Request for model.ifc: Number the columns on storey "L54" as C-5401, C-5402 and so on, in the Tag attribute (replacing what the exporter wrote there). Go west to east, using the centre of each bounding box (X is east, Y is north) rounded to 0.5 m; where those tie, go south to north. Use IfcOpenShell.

First a look at what the model holds.

```python
import ifcopenshell
import ifcopenshell.util.element
import ifcopenshell.util.placement

model = ifcopenshell.open("model.ifc")
print(model.schema)
storey = next(s for s in model.by_type("IfcBuildingStorey") if s.Name == "L54")
columns = [e for e in ifcopenshell.util.element.get_decomposition(storey) if e.is_a("IfcColumn")]
for e in sorted(columns, key=lambda e: e.id()):
    origin = ifcopenshell.util.placement.get_local_placement(e.ObjectPlacement)[:3, 3]
    print(e.id(), e.Tag, e.Name, origin.round(2) + 0.0, sep=" | ")
```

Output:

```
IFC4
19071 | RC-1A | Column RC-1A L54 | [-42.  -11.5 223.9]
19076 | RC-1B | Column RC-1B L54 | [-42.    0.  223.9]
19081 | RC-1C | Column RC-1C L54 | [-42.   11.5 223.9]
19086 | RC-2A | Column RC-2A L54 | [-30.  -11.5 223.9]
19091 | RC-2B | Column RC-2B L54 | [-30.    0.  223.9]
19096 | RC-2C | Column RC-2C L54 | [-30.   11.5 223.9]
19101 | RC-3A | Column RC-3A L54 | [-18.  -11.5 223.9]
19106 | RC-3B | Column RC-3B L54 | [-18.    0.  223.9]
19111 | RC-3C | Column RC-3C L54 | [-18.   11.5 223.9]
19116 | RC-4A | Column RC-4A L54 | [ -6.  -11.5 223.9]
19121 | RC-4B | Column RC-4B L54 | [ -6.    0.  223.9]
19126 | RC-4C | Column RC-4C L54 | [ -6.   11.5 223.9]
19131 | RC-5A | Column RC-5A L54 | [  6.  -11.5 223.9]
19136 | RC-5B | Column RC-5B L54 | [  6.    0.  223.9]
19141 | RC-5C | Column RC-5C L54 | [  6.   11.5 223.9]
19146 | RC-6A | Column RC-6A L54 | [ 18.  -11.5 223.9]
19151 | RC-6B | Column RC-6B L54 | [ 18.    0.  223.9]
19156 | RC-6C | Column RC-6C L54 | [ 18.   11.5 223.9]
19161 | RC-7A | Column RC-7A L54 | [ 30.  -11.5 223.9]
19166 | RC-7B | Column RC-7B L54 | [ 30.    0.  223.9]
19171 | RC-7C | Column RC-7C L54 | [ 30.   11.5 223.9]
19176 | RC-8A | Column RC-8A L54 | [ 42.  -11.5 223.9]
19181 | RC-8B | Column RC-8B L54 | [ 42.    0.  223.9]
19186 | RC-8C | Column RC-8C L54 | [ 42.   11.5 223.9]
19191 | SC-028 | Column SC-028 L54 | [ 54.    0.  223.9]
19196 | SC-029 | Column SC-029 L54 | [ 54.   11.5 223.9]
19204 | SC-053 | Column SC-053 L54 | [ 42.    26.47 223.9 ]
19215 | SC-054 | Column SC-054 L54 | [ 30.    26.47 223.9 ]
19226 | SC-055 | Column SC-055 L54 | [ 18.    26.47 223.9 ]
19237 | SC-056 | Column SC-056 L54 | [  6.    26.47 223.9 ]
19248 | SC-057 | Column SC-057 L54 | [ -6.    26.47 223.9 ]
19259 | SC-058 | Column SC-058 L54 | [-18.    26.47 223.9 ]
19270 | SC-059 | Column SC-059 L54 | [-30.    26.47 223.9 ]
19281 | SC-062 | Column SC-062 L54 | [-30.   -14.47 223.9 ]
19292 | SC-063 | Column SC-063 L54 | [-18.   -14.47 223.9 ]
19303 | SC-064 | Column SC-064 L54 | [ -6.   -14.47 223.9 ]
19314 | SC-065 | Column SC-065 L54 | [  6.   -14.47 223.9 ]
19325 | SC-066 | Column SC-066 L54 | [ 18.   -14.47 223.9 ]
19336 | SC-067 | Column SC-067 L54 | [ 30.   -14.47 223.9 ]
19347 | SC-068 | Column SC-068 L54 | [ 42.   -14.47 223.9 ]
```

```python
import ifcopenshell
import ifcopenshell.geom
import ifcopenshell.util.element
import ifcopenshell.util.shape

model = ifcopenshell.open("model.ifc")
settings = ifcopenshell.geom.settings()
settings.set("use-world-coords", True)


def centre(element):
    shape = ifcopenshell.geom.create_shape(settings, element)
    return ifcopenshell.util.shape.get_bbox_centroid(shape.geometry)


storey = next(s for s in model.by_type("IfcBuildingStorey") if s.Name == "L54")
columns = [e for e in ifcopenshell.util.element.get_decomposition(storey) if e.is_a("IfcColumn")]

# Insertion points can sit at a corner or the storey origin, so sort by the geometry (in metres).
centres = {e: centre(e) for e in columns}
columns.sort(key=lambda e: (round(centres[e][0] / 0.5), centres[e][1]))

for i, e in enumerate(columns, start=1):
    number = f"C-54{i:02d}"
    e.Tag = number
    print(e.id(), number)

model.write("model_updated.ifc")
```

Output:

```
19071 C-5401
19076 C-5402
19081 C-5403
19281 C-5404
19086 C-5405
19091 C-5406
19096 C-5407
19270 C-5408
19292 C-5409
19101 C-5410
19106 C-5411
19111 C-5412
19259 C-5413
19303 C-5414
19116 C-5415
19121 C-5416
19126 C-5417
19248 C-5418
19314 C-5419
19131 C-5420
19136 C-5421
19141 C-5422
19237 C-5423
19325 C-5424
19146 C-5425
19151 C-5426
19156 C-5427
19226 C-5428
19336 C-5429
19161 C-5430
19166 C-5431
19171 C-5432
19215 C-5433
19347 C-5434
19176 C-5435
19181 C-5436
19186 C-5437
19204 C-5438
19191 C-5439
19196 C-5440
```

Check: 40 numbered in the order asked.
